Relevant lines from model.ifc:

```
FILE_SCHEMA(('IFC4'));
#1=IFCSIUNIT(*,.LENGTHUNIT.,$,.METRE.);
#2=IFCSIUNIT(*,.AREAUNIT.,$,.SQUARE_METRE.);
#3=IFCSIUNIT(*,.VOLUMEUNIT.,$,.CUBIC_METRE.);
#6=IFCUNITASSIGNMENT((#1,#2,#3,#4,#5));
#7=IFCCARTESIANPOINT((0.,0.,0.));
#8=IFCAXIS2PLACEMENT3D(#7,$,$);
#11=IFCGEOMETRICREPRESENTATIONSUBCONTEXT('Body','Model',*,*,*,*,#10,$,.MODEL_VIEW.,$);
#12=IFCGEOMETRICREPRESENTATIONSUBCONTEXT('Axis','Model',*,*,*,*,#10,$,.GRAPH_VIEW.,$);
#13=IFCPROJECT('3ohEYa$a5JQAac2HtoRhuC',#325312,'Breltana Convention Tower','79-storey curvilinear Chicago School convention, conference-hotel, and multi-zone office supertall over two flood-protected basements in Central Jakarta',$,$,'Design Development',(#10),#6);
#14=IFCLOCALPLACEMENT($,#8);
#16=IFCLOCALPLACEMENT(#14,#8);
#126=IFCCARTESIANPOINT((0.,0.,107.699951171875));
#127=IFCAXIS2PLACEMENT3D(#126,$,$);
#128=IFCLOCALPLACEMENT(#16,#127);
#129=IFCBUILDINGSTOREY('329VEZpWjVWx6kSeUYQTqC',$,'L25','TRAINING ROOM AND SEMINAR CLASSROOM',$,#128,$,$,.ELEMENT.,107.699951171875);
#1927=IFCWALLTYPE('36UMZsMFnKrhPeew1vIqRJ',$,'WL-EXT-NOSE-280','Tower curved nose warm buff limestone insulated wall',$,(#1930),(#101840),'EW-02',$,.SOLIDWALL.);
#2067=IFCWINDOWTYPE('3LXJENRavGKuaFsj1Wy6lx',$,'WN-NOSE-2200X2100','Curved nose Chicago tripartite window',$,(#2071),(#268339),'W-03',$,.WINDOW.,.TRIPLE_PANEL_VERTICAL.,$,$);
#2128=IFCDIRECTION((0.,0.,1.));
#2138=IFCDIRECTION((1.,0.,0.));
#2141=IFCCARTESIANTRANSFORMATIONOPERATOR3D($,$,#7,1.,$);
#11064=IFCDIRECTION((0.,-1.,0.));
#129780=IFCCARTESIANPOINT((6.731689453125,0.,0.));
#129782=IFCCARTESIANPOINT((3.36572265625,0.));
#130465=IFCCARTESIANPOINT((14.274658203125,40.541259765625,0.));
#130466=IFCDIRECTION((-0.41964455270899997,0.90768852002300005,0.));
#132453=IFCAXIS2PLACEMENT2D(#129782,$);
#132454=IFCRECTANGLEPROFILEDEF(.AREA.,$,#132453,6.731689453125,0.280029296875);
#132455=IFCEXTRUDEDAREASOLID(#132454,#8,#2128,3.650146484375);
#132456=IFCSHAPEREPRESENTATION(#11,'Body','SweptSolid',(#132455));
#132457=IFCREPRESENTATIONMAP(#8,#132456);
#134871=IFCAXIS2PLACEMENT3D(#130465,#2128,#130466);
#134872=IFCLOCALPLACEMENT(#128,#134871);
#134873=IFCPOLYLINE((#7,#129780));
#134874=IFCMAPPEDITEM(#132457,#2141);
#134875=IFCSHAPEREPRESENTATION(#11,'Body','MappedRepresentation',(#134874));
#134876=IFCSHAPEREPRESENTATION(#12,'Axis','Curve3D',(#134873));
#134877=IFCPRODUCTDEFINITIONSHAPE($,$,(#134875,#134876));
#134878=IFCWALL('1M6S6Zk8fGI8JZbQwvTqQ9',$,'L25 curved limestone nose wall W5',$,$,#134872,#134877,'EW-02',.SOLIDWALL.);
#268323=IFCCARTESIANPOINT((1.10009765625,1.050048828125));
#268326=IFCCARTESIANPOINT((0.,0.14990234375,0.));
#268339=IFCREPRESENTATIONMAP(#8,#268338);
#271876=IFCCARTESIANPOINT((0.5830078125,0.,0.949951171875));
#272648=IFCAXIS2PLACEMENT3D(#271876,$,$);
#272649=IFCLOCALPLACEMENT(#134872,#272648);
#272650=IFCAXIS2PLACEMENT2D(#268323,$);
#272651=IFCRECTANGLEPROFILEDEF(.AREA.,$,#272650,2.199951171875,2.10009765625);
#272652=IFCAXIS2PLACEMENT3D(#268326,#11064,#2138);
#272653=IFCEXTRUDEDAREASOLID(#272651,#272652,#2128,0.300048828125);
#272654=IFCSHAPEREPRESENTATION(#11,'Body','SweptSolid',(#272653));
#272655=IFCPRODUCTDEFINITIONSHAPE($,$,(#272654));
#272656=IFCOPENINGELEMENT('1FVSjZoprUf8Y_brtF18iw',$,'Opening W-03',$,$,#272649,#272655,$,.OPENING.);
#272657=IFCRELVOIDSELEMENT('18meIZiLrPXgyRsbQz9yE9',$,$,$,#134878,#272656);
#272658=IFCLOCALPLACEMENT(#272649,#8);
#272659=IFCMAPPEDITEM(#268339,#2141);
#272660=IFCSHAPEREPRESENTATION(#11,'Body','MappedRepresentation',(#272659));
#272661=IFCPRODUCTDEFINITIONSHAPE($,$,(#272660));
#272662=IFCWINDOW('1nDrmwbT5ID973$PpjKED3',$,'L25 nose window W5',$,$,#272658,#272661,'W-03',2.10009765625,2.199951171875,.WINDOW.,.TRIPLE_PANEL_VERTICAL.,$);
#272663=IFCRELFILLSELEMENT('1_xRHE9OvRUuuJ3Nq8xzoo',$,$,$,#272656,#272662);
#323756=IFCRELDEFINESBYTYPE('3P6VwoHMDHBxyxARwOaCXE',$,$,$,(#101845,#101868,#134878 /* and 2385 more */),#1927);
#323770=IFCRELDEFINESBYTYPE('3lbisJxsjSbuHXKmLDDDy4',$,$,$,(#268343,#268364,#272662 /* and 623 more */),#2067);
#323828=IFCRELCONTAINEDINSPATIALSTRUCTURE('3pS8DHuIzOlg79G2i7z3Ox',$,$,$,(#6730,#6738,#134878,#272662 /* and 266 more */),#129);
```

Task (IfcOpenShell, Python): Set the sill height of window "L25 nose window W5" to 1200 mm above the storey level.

```python
import numpy as np
import ifcopenshell
import ifcopenshell.api.geometry
import ifcopenshell.geom
import ifcopenshell.util.element
import ifcopenshell.util.placement
import ifcopenshell.util.shape
import ifcopenshell.util.unit

model = ifcopenshell.open("model.ifc")
unit_scale = ifcopenshell.util.unit.calculate_unit_scale(model)

window = model.by_guid("1nDrmwbT5ID973$PpjKED3")
opening = window.FillsVoids[0].RelatingOpeningElement
storey = ifcopenshell.util.element.get_container(window, ifc_class="IfcBuildingStorey")
level = ifcopenshell.util.placement.get_local_placement(storey.ObjectPlacement)[2, 3]

# The opening's origin need not be at the sill, so measure its lowest point.
shape = ifcopenshell.geom.create_shape(ifcopenshell.geom.settings(), opening)
bottom = ifcopenshell.util.shape.get_shape_bottom_elevation(shape, shape.geometry) / unit_scale
dz = level + 1.2 - bottom

shift = np.array([0.0, 0.0, dz])
# The window is placed relative to its opening, so it follows when the opening moves.
matrix = ifcopenshell.util.placement.get_local_placement(opening.ObjectPlacement)
matrix[:3, 3] += shift
ifcopenshell.api.geometry.edit_object_placement(
    model, product=opening, matrix=matrix, is_si=False, should_transform_children=True
)

print(f"moved by {dz * unit_scale:+.3f} m")

model.write("model_edited.ifc")
```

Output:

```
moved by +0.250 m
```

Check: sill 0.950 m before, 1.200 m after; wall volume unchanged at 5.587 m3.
